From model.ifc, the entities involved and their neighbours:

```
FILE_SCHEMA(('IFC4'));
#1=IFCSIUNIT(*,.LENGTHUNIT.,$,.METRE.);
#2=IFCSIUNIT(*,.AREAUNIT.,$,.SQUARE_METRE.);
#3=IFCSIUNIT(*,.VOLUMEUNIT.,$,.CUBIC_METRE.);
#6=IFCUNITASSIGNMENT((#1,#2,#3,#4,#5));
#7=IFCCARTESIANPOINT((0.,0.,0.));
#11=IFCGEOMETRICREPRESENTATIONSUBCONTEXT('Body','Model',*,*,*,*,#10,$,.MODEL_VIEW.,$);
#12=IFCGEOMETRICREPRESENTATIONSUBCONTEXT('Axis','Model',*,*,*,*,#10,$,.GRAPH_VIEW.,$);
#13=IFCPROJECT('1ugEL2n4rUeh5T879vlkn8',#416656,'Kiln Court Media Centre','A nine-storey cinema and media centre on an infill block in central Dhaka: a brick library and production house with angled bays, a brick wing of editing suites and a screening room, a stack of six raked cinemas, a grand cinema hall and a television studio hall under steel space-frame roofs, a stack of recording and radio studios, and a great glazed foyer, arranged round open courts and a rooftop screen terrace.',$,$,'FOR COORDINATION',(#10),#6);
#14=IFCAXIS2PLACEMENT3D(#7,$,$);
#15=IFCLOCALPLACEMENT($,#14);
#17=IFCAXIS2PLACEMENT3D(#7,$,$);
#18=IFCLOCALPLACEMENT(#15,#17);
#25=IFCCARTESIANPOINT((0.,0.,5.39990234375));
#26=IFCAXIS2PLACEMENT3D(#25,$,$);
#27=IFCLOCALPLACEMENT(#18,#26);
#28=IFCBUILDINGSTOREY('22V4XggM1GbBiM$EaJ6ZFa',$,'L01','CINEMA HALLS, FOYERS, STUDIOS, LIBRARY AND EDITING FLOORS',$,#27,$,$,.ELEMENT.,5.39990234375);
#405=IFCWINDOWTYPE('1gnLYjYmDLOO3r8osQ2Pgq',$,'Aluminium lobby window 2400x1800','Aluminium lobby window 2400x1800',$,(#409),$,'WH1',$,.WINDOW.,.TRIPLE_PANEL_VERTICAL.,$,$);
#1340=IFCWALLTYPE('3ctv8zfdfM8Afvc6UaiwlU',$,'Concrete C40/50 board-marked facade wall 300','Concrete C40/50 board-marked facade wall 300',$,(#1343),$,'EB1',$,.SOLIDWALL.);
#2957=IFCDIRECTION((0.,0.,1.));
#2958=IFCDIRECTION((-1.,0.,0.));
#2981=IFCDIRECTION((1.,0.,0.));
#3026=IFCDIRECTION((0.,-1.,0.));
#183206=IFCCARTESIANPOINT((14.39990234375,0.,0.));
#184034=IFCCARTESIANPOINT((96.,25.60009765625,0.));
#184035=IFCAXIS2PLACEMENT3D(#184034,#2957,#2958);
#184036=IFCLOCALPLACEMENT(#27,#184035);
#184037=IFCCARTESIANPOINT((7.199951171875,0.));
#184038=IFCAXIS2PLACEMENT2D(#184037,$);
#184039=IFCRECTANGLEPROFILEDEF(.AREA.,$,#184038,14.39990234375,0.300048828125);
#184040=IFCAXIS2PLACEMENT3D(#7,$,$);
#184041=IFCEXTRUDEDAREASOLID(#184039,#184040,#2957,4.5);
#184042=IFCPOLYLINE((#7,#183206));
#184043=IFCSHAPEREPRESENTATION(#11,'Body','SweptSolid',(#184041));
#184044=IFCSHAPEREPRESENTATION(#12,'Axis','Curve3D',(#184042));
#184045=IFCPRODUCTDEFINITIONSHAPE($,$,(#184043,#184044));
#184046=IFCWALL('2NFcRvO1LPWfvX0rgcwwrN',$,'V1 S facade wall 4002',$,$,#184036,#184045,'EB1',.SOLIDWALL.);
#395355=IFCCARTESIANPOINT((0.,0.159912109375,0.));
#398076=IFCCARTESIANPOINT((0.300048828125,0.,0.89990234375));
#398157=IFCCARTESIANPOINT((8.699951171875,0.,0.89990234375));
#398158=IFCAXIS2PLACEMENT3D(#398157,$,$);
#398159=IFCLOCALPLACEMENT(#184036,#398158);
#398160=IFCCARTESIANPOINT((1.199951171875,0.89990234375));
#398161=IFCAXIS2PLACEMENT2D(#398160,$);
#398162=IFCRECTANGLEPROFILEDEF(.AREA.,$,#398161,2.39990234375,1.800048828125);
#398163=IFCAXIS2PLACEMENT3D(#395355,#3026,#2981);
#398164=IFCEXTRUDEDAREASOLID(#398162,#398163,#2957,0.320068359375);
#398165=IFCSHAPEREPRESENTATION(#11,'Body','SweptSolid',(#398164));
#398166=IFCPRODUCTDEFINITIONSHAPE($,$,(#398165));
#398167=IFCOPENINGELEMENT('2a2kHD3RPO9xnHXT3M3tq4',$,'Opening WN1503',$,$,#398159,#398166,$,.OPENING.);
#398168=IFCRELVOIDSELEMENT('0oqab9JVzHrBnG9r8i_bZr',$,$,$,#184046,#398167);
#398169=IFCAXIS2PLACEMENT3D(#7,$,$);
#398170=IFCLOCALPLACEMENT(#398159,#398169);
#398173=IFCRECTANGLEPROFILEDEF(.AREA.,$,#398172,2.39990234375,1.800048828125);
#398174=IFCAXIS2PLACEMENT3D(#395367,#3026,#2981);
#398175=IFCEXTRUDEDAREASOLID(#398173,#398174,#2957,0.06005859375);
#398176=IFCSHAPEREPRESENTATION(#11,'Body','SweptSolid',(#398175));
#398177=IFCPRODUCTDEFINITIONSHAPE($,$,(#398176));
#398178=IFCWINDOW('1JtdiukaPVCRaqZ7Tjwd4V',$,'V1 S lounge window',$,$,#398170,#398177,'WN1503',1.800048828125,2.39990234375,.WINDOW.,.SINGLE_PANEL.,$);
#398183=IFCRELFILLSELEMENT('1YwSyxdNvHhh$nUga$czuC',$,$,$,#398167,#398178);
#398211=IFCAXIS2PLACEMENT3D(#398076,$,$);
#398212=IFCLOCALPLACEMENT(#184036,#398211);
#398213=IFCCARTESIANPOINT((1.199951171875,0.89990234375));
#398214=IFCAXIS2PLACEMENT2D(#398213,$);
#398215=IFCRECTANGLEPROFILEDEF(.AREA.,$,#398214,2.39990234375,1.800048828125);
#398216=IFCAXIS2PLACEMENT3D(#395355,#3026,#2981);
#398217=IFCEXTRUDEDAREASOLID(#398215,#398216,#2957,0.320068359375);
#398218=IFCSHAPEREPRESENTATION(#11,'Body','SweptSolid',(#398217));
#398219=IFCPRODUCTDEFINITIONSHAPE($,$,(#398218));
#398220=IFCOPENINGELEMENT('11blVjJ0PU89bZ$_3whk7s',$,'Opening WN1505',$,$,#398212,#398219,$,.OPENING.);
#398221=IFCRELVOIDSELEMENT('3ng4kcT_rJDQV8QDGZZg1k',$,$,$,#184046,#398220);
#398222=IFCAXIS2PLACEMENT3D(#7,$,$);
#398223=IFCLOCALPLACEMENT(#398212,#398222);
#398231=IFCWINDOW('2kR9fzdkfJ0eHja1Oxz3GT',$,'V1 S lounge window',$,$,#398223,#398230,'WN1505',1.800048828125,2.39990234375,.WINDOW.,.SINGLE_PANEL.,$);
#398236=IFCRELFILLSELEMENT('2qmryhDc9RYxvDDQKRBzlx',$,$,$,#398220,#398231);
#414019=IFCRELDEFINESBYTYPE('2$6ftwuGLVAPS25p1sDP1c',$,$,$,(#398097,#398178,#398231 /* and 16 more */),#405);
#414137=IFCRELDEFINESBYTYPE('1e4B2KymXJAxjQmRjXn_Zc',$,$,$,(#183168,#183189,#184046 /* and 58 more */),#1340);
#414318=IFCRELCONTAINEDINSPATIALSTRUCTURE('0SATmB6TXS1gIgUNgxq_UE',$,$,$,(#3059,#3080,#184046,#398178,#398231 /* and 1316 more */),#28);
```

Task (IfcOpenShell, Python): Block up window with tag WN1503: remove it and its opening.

```python
import ifcopenshell
import ifcopenshell.api.feature
import ifcopenshell.api.root
import ifcopenshell.geom
import ifcopenshell.util.shape

model = ifcopenshell.open("model.ifc")
settings = ifcopenshell.geom.settings()


def volume(element):
    """Net volume in cubic metres, openings subtracted."""
    shape = ifcopenshell.geom.create_shape(settings, element)
    return ifcopenshell.util.shape.get_volume(shape.geometry)


window = model.by_guid("1JtdiukaPVCRaqZ7Tjwd4V")
opening = window.FillsVoids[0].RelatingOpeningElement
wall = opening.VoidsElements[0].RelatingBuildingElement
before = volume(wall)

ifcopenshell.api.root.remove_product(model, product=window)
ifcopenshell.api.feature.remove_feature(model, feature=opening)

after = volume(wall)

print(f"wall volume {before:.3f} -> {after:.3f} m3")

model.write("model_v2.ifc")
```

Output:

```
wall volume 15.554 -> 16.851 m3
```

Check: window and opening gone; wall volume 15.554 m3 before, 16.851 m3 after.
